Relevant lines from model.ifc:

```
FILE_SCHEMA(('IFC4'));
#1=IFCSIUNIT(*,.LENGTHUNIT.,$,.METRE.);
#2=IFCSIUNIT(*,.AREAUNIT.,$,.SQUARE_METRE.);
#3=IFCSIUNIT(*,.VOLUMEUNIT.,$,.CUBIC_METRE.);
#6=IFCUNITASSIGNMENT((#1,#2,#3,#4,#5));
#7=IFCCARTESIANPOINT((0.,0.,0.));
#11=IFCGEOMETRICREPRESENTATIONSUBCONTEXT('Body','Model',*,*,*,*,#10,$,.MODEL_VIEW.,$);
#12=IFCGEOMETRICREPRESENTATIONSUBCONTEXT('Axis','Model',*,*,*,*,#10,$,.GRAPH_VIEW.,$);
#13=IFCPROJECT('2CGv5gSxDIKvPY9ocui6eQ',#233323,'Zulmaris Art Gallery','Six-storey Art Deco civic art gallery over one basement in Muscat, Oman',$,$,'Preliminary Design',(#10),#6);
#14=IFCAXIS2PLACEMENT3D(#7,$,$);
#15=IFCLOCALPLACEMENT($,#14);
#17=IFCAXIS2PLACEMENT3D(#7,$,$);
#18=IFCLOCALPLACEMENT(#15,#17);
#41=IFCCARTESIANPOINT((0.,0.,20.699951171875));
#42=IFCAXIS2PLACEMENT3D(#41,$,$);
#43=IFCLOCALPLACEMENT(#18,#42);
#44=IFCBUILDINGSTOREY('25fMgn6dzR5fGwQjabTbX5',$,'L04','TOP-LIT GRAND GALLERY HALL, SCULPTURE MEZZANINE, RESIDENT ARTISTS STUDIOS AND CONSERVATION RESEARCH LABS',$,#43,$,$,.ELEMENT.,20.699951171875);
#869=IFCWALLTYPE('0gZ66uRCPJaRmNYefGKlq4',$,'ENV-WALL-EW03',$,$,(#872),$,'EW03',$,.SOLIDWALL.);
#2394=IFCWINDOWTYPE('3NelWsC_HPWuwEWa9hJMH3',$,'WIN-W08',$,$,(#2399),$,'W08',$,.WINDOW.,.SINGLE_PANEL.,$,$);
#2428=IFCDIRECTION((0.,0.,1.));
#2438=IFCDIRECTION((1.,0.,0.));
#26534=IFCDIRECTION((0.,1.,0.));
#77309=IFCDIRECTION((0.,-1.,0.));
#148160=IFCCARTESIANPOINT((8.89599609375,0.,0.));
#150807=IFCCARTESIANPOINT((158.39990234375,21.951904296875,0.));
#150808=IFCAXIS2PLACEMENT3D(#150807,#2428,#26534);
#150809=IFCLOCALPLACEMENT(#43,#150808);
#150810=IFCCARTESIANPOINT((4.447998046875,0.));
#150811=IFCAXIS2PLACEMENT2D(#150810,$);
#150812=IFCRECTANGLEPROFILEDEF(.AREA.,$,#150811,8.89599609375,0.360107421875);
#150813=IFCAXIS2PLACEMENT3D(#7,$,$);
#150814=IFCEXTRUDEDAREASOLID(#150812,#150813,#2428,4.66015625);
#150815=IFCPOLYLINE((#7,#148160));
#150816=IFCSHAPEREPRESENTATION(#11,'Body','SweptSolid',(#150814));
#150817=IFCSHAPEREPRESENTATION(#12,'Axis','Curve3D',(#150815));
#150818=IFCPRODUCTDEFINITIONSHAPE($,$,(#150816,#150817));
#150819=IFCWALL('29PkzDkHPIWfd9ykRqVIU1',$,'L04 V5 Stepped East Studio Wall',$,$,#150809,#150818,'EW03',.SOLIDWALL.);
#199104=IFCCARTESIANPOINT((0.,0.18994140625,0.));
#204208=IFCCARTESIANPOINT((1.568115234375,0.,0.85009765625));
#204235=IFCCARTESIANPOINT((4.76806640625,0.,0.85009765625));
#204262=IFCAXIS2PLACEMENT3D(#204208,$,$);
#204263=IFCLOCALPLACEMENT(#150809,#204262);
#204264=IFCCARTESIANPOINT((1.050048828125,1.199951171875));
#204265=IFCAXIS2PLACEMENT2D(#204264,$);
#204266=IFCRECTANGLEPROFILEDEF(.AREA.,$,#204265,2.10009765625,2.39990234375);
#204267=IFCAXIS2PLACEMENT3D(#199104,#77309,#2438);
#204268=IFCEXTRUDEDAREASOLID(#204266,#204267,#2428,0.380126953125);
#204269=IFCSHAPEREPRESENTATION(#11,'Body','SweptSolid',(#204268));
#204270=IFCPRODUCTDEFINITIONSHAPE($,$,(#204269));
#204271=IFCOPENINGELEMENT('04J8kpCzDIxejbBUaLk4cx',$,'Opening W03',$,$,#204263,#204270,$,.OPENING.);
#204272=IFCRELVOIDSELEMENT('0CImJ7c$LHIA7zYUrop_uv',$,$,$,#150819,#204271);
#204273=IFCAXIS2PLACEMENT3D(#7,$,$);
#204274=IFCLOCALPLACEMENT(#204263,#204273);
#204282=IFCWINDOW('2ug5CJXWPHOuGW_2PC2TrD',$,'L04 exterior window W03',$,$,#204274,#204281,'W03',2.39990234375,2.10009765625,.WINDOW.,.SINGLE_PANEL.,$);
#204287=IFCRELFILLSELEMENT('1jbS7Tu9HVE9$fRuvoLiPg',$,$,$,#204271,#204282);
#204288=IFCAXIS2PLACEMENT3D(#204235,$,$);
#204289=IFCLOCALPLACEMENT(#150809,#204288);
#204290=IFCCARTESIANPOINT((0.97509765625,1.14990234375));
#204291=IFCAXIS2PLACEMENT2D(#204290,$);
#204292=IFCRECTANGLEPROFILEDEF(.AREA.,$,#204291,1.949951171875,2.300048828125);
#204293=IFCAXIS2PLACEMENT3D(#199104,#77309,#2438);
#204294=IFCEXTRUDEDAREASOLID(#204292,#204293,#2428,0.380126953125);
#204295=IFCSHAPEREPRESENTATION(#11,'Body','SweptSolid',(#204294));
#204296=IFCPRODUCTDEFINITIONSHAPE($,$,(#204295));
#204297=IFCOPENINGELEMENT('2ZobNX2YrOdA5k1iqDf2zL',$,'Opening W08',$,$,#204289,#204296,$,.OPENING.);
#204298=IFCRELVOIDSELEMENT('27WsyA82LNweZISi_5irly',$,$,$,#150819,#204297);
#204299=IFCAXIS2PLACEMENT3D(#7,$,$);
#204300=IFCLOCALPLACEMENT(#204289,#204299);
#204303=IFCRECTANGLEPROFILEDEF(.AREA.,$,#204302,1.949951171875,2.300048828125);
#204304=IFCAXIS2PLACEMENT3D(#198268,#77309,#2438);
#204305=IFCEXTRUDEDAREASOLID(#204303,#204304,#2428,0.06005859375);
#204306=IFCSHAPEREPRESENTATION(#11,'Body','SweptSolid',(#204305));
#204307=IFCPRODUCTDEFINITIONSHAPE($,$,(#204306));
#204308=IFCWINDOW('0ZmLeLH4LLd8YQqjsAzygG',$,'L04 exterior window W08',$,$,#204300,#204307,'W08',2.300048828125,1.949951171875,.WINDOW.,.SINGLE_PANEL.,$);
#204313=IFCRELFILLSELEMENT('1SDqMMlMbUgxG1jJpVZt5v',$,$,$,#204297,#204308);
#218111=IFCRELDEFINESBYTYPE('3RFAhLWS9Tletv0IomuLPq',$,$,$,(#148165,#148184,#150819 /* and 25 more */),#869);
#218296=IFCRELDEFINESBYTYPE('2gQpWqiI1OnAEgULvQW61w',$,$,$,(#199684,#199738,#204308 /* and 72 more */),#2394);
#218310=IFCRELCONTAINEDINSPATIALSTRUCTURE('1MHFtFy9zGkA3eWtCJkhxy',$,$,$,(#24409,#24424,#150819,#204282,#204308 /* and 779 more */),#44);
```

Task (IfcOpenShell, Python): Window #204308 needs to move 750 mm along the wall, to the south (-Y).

```python
import ifcopenshell
import ifcopenshell.api.geometry
import ifcopenshell.util.placement
import ifcopenshell.util.unit

model = ifcopenshell.open("model.ifc")
unit_scale = ifcopenshell.util.unit.calculate_unit_scale(model)

window = model.by_guid("0ZmLeLH4LLd8YQqjsAzygG")
opening = window.FillsVoids[0].RelatingOpeningElement
wall = opening.VoidsElements[0].RelatingBuildingElement

wall_matrix = ifcopenshell.util.placement.get_local_placement(wall.ObjectPlacement)
shift = wall_matrix[:3, 0] * -0.75 / unit_scale
before = ifcopenshell.util.placement.get_local_placement(window.ObjectPlacement)[:3, 3].copy()

# The window is placed relative to its opening, so it follows when the opening moves.
matrix = ifcopenshell.util.placement.get_local_placement(opening.ObjectPlacement)
matrix[:3, 3] += shift
ifcopenshell.api.geometry.edit_object_placement(
    model, product=opening, matrix=matrix, is_si=False, should_transform_children=True
)

after = ifcopenshell.util.placement.get_local_placement(window.ObjectPlacement)[:3, 3]
print("window moved by", (after - before).round(3) + 0.0)

model.write("model_edited.ifc")
```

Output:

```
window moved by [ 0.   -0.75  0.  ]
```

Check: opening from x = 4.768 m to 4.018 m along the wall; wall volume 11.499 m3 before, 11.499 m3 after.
